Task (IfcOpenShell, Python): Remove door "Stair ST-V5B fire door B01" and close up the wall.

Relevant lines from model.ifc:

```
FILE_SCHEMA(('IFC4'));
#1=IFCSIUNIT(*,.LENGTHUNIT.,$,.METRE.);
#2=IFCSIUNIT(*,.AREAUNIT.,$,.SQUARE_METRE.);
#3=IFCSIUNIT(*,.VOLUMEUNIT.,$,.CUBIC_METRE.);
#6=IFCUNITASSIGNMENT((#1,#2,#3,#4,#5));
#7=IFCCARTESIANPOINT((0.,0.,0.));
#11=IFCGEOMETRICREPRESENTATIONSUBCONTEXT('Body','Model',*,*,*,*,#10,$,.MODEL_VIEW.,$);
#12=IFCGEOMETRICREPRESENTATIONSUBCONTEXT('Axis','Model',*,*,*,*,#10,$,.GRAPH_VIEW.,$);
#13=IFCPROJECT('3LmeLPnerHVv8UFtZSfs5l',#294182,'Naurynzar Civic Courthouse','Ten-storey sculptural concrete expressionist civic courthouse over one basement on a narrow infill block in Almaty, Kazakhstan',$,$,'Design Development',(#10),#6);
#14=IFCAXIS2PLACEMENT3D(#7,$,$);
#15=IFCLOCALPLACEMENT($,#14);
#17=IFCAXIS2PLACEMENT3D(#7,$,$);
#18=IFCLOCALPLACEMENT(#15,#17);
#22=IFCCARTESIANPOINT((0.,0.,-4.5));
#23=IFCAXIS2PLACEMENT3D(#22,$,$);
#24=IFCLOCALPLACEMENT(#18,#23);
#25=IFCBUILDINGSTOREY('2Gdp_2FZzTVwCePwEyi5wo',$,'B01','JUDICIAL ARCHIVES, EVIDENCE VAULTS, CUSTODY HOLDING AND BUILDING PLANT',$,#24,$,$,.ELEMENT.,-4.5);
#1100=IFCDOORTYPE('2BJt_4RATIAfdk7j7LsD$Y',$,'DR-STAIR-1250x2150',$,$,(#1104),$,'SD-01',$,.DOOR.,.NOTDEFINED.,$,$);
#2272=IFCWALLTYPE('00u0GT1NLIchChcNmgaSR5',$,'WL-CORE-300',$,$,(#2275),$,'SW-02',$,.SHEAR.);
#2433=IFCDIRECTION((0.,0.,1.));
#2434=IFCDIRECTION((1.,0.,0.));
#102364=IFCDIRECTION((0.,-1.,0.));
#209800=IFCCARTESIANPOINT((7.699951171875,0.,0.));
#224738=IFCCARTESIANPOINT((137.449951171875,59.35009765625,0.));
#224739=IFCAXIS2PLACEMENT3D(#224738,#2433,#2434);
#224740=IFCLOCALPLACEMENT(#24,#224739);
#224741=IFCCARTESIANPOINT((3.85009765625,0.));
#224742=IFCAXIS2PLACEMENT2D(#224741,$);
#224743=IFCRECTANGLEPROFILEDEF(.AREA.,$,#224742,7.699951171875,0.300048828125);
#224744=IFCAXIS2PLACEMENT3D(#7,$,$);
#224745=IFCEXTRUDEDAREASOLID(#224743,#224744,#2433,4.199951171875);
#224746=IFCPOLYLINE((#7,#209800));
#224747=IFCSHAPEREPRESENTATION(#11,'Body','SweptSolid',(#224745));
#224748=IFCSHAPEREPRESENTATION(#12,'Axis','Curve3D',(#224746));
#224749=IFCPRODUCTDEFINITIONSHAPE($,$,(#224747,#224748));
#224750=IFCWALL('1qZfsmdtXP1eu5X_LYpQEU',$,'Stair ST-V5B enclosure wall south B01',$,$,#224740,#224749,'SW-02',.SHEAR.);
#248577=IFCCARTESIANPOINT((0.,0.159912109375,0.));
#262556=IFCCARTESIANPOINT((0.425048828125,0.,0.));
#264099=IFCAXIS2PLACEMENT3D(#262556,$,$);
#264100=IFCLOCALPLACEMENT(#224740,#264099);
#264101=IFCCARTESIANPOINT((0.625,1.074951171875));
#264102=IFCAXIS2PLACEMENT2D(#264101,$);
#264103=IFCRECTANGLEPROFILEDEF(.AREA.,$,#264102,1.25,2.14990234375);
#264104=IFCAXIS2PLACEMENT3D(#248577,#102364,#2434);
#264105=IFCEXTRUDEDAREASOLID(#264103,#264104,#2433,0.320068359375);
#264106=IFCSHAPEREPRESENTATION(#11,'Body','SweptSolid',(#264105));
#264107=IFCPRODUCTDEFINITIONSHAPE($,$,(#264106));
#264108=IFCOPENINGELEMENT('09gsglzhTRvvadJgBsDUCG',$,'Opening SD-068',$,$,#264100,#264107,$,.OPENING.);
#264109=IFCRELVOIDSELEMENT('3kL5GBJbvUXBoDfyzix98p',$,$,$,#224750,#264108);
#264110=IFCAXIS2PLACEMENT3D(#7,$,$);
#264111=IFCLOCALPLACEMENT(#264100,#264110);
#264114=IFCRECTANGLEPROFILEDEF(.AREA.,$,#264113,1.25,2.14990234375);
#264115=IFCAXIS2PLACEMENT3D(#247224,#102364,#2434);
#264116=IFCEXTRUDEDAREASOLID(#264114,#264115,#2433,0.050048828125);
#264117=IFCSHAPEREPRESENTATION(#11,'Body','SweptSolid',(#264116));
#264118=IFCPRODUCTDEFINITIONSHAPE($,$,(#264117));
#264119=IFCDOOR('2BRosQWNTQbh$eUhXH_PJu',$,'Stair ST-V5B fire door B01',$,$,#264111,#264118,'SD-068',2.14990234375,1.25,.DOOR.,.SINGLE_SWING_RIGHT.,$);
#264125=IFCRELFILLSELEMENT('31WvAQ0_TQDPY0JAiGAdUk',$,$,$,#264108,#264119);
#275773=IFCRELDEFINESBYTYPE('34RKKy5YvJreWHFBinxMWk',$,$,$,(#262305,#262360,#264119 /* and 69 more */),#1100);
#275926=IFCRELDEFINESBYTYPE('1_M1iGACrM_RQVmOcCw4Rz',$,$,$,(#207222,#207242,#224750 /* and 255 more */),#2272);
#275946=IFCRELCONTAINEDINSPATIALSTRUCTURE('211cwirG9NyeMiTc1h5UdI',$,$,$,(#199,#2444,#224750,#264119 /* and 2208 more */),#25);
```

```python
import ifcopenshell
import ifcopenshell.api.feature
import ifcopenshell.api.root
import ifcopenshell.geom
import ifcopenshell.util.shape

model = ifcopenshell.open("model.ifc")
settings = ifcopenshell.geom.settings()


def volume(element):
    """Net volume in cubic metres, openings subtracted."""
    shape = ifcopenshell.geom.create_shape(settings, element)
    return ifcopenshell.util.shape.get_volume(shape.geometry)


door = model.by_guid("2BRosQWNTQbh$eUhXH_PJu")
opening = door.FillsVoids[0].RelatingOpeningElement
wall = opening.VoidsElements[0].RelatingBuildingElement
before = volume(wall)

ifcopenshell.api.root.remove_product(model, product=door)
ifcopenshell.api.feature.remove_feature(model, feature=opening)

after = volume(wall)

print(f"wall volume {before:.3f} -> {after:.3f} m3")

model.write("model_v2.ifc")
```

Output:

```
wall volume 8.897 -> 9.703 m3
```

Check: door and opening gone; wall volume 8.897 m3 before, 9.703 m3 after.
